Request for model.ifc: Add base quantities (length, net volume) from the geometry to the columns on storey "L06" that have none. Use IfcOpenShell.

First a look at what the model holds.

```python
import ifcopenshell
import ifcopenshell.util.element
import ifcopenshell.util.unit

model = ifcopenshell.open("model.ifc")
print(model.schema)
for unit_type in ("LENGTHUNIT", "AREAUNIT", "VOLUMEUNIT"):
    print(unit_type, ifcopenshell.util.unit.calculate_unit_scale(model, unit_type))
storey = next(s for s in model.by_type("IfcBuildingStorey") if s.Name == "L06")
columns = [e for e in ifcopenshell.util.element.get_decomposition(storey) if e.is_a("IfcColumn")]
for e in sorted(columns, key=lambda e: e.id()):
    print(e.id(), e.is_a(), e.Name, list(ifcopenshell.util.element.get_psets(e, qtos_only=True)), sep=" | ")
```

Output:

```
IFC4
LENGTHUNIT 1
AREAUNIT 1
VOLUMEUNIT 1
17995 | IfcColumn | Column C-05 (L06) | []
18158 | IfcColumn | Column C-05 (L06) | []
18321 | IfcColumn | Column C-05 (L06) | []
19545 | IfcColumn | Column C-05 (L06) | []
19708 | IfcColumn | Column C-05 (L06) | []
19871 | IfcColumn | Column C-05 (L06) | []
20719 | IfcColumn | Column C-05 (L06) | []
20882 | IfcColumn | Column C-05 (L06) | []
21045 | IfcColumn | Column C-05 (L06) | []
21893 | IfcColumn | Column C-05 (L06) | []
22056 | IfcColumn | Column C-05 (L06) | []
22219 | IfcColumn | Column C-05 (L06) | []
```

```python
import ifcopenshell
import ifcopenshell.api.pset
import ifcopenshell.geom
import ifcopenshell.util.element
import ifcopenshell.util.shape
import ifcopenshell.util.unit

model = ifcopenshell.open("model.ifc")
unit_scale = ifcopenshell.util.unit.calculate_unit_scale(model)
volume_scale = ifcopenshell.util.unit.calculate_unit_scale(model, "VOLUMEUNIT")
settings = ifcopenshell.geom.settings()

storey = next(s for s in model.by_type("IfcBuildingStorey") if s.Name == "L06")
columns = [e for e in ifcopenshell.util.element.get_decomposition(storey) if e.is_a("IfcColumn")]

for e in sorted(columns, key=lambda e: e.id()):
    if ifcopenshell.util.element.get_psets(e, qtos_only=True, should_inherit=False):
        continue
    # Geometry comes back in metres, in the element's own axes.
    shape = ifcopenshell.geom.create_shape(settings, e)
    values = {
        "Length": ifcopenshell.util.shape.get_z(shape.geometry) / unit_scale,
        "NetVolume": ifcopenshell.util.shape.get_volume(shape.geometry) / volume_scale,
    }
    qto = ifcopenshell.api.pset.add_qto(model, product=e, name="Qto_ColumnBaseQuantities")
    ifcopenshell.api.pset.edit_qto(model, qto=qto, properties=values)
    print(e.id(), {k: round(v, 3) for k, v in values.items()})

model.write("model_updated.ifc")
```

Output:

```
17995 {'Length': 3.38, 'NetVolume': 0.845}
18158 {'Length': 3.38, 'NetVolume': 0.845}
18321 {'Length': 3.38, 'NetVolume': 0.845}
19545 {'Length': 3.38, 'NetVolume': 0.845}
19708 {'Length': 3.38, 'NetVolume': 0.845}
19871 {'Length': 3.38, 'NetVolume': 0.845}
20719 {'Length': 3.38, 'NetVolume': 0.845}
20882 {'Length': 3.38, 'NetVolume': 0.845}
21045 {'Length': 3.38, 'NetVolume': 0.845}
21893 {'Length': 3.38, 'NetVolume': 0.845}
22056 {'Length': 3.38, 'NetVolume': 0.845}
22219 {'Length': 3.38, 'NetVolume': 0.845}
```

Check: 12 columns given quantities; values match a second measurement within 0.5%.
